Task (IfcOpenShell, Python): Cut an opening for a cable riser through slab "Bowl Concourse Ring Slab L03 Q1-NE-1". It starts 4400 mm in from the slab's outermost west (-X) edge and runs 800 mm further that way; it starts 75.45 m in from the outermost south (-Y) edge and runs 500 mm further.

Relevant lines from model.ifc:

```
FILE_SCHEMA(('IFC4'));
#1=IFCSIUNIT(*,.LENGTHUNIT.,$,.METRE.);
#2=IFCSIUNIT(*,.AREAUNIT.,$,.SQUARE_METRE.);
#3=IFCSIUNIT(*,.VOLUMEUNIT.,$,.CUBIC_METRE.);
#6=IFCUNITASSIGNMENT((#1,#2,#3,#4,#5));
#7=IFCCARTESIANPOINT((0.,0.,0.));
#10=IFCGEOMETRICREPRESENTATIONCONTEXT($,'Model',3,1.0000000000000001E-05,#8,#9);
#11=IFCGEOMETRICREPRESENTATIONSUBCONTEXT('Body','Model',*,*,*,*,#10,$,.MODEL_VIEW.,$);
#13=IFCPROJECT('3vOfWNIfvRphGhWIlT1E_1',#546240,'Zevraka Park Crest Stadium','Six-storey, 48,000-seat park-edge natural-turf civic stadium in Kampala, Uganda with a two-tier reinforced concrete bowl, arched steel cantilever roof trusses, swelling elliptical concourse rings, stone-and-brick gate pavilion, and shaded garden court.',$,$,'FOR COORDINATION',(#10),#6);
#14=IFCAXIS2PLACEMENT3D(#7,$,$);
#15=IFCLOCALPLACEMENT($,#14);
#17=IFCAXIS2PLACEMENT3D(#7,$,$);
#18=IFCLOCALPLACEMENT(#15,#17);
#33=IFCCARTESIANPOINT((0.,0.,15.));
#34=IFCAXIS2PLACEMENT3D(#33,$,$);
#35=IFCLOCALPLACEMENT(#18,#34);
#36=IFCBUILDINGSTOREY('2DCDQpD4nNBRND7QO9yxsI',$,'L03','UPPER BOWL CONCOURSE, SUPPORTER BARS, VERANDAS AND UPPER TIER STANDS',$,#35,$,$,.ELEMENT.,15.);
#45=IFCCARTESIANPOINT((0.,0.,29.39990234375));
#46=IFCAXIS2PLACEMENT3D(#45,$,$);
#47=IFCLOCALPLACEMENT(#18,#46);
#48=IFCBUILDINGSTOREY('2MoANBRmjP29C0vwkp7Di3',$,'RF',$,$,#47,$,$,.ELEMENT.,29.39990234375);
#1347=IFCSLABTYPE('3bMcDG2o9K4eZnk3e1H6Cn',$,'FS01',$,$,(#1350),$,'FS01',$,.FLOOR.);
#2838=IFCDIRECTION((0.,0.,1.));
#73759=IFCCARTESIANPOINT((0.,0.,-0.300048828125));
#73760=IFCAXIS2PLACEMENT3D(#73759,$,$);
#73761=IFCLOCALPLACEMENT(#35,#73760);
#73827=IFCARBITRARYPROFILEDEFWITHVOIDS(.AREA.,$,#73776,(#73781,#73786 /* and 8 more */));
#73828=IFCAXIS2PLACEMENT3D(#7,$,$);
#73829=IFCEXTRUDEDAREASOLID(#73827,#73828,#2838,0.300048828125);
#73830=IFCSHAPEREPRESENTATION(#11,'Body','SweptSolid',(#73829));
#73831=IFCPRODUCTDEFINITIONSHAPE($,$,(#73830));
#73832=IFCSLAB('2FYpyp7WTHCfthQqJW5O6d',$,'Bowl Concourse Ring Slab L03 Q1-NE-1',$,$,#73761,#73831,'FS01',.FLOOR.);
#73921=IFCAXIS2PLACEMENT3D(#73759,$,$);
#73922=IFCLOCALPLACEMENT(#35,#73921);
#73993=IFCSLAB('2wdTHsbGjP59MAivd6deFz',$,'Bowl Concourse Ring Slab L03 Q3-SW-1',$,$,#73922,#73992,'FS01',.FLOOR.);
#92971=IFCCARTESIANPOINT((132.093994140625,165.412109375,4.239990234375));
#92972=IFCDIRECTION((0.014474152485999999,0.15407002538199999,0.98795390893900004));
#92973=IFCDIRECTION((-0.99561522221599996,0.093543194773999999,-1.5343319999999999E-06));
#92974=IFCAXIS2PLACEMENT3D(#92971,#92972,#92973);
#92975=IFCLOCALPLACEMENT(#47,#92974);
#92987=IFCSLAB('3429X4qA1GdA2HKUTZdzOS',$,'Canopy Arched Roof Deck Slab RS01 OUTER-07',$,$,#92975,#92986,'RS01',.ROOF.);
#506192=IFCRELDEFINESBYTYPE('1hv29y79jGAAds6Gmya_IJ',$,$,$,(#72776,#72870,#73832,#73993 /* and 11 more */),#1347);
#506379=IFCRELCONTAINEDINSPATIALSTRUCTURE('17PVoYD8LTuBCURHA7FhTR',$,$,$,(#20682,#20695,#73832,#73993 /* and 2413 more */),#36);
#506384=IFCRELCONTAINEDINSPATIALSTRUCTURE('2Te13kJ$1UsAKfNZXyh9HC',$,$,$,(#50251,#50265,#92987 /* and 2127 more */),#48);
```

```python
import numpy as np
import ifcopenshell
import ifcopenshell.api.feature
import ifcopenshell.api.geometry
import ifcopenshell.api.root
import ifcopenshell.geom
import ifcopenshell.util.placement
import ifcopenshell.util.representation
import ifcopenshell.util.shape
import ifcopenshell.util.unit

model = ifcopenshell.open("model.ifc")
unit_scale = ifcopenshell.util.unit.calculate_unit_scale(model)
settings = ifcopenshell.geom.settings()


def volume(element):
    """Net volume in cubic metres, openings subtracted."""
    shape = ifcopenshell.geom.create_shape(settings, element)
    return ifcopenshell.util.shape.get_volume(shape.geometry)


slab = model.by_id(73832)
before = volume(slab)

# Extent in the slab's own axes, in metres. The edges named are its -X and -Y sides.
slab_shape = ifcopenshell.geom.create_shape(settings, slab)
vertices = ifcopenshell.util.shape.get_vertices(slab_shape.geometry)
x_min, y_min, bottom = vertices.min(axis=0)
top = vertices[:, 2].max()

opening = ifcopenshell.api.root.create_entity(model, ifc_class="IfcOpeningElement", name="Cable riser opening", predefined_type="OPENING")
context = ifcopenshell.util.representation.get_context(model, "Model", "Body", "MODEL_VIEW")
width, depth = 0.8, 0.5
outline = [(0.0, 0.0), (width, 0.0), (width, depth), (0.0, depth), (0.0, 0.0)]
# Overshoot both faces by 50 mm so the cut is clean.
shape = ifcopenshell.api.geometry.add_slab_representation(
    model, context=context, depth=top - bottom + 0.1, polyline=outline
)
ifcopenshell.api.geometry.assign_representation(model, product=opening, representation=shape)

matrix = ifcopenshell.util.placement.get_local_placement(slab.ObjectPlacement)
matrix[:, 3] = matrix @ np.append(np.array([x_min + 4.4, y_min + 75.45, bottom - 0.05]) / unit_scale, 1.0)
ifcopenshell.api.geometry.edit_object_placement(model, product=opening, matrix=matrix, is_si=False)
ifcopenshell.api.feature.add_feature(model, feature=opening, element=slab)

after = volume(slab)

print(f"slab volume {before:.3f} -> {after:.3f} m3")

model.write("model-out.ifc")
```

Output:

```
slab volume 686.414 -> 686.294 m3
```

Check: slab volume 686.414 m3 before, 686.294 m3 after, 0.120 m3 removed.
